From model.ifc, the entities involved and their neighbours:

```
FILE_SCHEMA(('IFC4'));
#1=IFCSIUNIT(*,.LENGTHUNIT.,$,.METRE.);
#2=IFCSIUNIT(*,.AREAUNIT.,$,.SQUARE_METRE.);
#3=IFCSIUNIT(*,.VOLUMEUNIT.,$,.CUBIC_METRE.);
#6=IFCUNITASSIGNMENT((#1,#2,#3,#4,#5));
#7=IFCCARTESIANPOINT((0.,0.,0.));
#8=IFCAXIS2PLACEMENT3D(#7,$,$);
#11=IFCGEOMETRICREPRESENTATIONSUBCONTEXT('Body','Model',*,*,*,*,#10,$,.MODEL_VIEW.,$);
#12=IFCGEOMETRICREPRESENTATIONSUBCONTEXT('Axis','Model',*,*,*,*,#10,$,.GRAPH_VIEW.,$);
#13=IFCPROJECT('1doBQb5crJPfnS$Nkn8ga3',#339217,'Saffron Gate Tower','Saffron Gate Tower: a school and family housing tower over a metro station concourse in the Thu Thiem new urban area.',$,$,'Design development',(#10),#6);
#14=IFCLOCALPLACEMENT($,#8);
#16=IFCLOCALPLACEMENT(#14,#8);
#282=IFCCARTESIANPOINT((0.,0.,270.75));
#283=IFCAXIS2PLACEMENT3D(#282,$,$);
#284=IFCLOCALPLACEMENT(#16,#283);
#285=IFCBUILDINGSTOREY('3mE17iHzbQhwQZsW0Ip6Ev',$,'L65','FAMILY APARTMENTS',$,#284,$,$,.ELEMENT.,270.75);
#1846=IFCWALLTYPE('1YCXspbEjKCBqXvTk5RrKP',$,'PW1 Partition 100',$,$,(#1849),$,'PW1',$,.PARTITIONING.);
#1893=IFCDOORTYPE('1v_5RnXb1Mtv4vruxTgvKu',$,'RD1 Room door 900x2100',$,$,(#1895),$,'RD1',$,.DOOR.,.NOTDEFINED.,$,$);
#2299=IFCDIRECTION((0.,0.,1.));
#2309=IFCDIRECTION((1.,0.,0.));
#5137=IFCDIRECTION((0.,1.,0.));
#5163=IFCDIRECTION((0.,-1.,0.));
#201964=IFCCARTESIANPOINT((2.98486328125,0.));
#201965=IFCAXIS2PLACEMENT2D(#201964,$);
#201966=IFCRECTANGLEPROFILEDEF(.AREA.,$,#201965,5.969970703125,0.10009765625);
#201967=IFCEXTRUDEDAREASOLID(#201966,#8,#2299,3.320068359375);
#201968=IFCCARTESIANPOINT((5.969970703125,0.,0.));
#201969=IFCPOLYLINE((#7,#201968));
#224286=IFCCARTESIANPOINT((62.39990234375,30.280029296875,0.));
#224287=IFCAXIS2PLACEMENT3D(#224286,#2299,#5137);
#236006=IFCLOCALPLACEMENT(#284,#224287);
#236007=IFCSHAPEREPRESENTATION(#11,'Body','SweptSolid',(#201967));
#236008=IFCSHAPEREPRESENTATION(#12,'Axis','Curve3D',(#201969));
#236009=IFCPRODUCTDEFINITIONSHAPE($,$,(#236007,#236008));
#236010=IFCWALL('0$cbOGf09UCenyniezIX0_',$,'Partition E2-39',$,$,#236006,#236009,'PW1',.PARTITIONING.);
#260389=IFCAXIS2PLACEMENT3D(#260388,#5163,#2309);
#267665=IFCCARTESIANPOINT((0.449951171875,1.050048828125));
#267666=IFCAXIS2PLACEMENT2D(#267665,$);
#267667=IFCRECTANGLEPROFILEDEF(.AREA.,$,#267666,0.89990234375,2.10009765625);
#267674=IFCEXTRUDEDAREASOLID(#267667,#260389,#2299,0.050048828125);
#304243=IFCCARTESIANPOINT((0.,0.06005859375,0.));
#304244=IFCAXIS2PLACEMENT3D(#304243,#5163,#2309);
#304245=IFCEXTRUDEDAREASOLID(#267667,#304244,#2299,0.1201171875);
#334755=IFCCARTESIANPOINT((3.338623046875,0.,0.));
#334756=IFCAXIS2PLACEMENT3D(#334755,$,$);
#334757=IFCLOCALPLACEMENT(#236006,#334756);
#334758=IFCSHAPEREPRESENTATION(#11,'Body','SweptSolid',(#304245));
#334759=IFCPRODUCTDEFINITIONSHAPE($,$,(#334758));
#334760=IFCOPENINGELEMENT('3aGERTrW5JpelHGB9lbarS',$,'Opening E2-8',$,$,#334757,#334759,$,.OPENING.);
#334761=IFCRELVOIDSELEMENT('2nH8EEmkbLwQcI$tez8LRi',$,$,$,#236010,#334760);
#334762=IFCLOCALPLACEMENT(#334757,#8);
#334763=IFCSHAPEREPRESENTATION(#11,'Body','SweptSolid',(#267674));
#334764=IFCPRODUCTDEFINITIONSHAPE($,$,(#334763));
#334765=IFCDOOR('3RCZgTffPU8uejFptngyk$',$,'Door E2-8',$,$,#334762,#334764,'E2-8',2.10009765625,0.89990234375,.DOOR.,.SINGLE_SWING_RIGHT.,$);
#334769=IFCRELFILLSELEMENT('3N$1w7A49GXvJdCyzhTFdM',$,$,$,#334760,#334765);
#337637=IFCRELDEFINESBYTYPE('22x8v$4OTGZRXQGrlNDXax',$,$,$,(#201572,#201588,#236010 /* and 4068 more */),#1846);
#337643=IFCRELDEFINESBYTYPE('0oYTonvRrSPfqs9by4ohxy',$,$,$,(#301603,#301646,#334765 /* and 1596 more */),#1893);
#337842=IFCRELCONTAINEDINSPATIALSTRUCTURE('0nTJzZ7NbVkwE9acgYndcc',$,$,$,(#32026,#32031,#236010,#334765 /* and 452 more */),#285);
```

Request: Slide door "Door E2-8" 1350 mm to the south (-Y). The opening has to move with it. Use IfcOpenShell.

```python
import ifcopenshell
import ifcopenshell.api.geometry
import ifcopenshell.util.placement
import ifcopenshell.util.unit

model = ifcopenshell.open("model.ifc")
unit_scale = ifcopenshell.util.unit.calculate_unit_scale(model)

door = model.by_guid("3RCZgTffPU8uejFptngyk$")
opening = door.FillsVoids[0].RelatingOpeningElement
wall = opening.VoidsElements[0].RelatingBuildingElement

wall_matrix = ifcopenshell.util.placement.get_local_placement(wall.ObjectPlacement)
shift = wall_matrix[:3, 0] * -1.35 / unit_scale
before = ifcopenshell.util.placement.get_local_placement(door.ObjectPlacement)[:3, 3].copy()

# The door is placed relative to its opening, so it follows when the opening moves.
matrix = ifcopenshell.util.placement.get_local_placement(opening.ObjectPlacement)
matrix[:3, 3] += shift
ifcopenshell.api.geometry.edit_object_placement(
    model, product=opening, matrix=matrix, is_si=False, should_transform_children=True
)

after = ifcopenshell.util.placement.get_local_placement(door.ObjectPlacement)[:3, 3]
print("door moved by", (after - before).round(3) + 0.0)

model.write("model-out.ifc")
```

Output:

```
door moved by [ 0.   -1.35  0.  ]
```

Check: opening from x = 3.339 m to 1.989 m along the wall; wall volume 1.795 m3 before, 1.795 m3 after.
